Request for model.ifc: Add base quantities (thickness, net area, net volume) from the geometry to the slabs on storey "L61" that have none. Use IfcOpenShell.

First a look at what the model holds.

```python
import ifcopenshell
import ifcopenshell.util.element
import ifcopenshell.util.unit

model = ifcopenshell.open("model.ifc")
print(model.schema)
for unit_type in ("LENGTHUNIT", "AREAUNIT", "VOLUMEUNIT"):
    print(unit_type, ifcopenshell.util.unit.calculate_unit_scale(model, unit_type))
storey = next(s for s in model.by_type("IfcBuildingStorey") if s.Name == "L61")
slabs = [e for e in ifcopenshell.util.element.get_decomposition(storey) if e.is_a("IfcSlab")]
for e in sorted(slabs, key=lambda e: e.id()):
    print(e.id(), e.is_a(), e.Name, list(ifcopenshell.util.element.get_psets(e, qtos_only=True)), sep=" | ")
```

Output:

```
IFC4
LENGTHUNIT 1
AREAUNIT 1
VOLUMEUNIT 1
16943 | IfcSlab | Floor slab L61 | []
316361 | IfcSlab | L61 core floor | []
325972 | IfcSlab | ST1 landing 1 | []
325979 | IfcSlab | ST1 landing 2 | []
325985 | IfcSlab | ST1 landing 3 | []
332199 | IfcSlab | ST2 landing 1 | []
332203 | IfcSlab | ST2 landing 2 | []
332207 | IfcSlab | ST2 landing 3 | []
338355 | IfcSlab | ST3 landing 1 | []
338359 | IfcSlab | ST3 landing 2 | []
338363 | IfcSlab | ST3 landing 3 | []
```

```python
import ifcopenshell
import ifcopenshell.api.pset
import ifcopenshell.geom
import ifcopenshell.util.element
import ifcopenshell.util.shape
import ifcopenshell.util.unit

model = ifcopenshell.open("model.ifc")
unit_scale = ifcopenshell.util.unit.calculate_unit_scale(model)
area_scale = ifcopenshell.util.unit.calculate_unit_scale(model, "AREAUNIT")
volume_scale = ifcopenshell.util.unit.calculate_unit_scale(model, "VOLUMEUNIT")
settings = ifcopenshell.geom.settings()

storey = next(s for s in model.by_type("IfcBuildingStorey") if s.Name == "L61")
slabs = [e for e in ifcopenshell.util.element.get_decomposition(storey) if e.is_a("IfcSlab")]

for e in sorted(slabs, key=lambda e: e.id()):
    if ifcopenshell.util.element.get_psets(e, qtos_only=True, should_inherit=False):
        continue
    # Geometry comes back in metres, in the element's own axes.
    shape = ifcopenshell.geom.create_shape(settings, e)
    values = {
        "Width": ifcopenshell.util.shape.get_z(shape.geometry) / unit_scale,
        "NetArea": ifcopenshell.util.shape.get_footprint_area(shape.geometry) / area_scale,
        "NetVolume": ifcopenshell.util.shape.get_volume(shape.geometry) / volume_scale,
    }
    qto = ifcopenshell.api.pset.add_qto(model, product=e, name="Qto_SlabBaseQuantities")
    ifcopenshell.api.pset.edit_qto(model, qto=qto, properties=values)
    print(e.id(), {k: round(v, 3) for k, v in values.items()})

model.write("model_edited.ifc")
```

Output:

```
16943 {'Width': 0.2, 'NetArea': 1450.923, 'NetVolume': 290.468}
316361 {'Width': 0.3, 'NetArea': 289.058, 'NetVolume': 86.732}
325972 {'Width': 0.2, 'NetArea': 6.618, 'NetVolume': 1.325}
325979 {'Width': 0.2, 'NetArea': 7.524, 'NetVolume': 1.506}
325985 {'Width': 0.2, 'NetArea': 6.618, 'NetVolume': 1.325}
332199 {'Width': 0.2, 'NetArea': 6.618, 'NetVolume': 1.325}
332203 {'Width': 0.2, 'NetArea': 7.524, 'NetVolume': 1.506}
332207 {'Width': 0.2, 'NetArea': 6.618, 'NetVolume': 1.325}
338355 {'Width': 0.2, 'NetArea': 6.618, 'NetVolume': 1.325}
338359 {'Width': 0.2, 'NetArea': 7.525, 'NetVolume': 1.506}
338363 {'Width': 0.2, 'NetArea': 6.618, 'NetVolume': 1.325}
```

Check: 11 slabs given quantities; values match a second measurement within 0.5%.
